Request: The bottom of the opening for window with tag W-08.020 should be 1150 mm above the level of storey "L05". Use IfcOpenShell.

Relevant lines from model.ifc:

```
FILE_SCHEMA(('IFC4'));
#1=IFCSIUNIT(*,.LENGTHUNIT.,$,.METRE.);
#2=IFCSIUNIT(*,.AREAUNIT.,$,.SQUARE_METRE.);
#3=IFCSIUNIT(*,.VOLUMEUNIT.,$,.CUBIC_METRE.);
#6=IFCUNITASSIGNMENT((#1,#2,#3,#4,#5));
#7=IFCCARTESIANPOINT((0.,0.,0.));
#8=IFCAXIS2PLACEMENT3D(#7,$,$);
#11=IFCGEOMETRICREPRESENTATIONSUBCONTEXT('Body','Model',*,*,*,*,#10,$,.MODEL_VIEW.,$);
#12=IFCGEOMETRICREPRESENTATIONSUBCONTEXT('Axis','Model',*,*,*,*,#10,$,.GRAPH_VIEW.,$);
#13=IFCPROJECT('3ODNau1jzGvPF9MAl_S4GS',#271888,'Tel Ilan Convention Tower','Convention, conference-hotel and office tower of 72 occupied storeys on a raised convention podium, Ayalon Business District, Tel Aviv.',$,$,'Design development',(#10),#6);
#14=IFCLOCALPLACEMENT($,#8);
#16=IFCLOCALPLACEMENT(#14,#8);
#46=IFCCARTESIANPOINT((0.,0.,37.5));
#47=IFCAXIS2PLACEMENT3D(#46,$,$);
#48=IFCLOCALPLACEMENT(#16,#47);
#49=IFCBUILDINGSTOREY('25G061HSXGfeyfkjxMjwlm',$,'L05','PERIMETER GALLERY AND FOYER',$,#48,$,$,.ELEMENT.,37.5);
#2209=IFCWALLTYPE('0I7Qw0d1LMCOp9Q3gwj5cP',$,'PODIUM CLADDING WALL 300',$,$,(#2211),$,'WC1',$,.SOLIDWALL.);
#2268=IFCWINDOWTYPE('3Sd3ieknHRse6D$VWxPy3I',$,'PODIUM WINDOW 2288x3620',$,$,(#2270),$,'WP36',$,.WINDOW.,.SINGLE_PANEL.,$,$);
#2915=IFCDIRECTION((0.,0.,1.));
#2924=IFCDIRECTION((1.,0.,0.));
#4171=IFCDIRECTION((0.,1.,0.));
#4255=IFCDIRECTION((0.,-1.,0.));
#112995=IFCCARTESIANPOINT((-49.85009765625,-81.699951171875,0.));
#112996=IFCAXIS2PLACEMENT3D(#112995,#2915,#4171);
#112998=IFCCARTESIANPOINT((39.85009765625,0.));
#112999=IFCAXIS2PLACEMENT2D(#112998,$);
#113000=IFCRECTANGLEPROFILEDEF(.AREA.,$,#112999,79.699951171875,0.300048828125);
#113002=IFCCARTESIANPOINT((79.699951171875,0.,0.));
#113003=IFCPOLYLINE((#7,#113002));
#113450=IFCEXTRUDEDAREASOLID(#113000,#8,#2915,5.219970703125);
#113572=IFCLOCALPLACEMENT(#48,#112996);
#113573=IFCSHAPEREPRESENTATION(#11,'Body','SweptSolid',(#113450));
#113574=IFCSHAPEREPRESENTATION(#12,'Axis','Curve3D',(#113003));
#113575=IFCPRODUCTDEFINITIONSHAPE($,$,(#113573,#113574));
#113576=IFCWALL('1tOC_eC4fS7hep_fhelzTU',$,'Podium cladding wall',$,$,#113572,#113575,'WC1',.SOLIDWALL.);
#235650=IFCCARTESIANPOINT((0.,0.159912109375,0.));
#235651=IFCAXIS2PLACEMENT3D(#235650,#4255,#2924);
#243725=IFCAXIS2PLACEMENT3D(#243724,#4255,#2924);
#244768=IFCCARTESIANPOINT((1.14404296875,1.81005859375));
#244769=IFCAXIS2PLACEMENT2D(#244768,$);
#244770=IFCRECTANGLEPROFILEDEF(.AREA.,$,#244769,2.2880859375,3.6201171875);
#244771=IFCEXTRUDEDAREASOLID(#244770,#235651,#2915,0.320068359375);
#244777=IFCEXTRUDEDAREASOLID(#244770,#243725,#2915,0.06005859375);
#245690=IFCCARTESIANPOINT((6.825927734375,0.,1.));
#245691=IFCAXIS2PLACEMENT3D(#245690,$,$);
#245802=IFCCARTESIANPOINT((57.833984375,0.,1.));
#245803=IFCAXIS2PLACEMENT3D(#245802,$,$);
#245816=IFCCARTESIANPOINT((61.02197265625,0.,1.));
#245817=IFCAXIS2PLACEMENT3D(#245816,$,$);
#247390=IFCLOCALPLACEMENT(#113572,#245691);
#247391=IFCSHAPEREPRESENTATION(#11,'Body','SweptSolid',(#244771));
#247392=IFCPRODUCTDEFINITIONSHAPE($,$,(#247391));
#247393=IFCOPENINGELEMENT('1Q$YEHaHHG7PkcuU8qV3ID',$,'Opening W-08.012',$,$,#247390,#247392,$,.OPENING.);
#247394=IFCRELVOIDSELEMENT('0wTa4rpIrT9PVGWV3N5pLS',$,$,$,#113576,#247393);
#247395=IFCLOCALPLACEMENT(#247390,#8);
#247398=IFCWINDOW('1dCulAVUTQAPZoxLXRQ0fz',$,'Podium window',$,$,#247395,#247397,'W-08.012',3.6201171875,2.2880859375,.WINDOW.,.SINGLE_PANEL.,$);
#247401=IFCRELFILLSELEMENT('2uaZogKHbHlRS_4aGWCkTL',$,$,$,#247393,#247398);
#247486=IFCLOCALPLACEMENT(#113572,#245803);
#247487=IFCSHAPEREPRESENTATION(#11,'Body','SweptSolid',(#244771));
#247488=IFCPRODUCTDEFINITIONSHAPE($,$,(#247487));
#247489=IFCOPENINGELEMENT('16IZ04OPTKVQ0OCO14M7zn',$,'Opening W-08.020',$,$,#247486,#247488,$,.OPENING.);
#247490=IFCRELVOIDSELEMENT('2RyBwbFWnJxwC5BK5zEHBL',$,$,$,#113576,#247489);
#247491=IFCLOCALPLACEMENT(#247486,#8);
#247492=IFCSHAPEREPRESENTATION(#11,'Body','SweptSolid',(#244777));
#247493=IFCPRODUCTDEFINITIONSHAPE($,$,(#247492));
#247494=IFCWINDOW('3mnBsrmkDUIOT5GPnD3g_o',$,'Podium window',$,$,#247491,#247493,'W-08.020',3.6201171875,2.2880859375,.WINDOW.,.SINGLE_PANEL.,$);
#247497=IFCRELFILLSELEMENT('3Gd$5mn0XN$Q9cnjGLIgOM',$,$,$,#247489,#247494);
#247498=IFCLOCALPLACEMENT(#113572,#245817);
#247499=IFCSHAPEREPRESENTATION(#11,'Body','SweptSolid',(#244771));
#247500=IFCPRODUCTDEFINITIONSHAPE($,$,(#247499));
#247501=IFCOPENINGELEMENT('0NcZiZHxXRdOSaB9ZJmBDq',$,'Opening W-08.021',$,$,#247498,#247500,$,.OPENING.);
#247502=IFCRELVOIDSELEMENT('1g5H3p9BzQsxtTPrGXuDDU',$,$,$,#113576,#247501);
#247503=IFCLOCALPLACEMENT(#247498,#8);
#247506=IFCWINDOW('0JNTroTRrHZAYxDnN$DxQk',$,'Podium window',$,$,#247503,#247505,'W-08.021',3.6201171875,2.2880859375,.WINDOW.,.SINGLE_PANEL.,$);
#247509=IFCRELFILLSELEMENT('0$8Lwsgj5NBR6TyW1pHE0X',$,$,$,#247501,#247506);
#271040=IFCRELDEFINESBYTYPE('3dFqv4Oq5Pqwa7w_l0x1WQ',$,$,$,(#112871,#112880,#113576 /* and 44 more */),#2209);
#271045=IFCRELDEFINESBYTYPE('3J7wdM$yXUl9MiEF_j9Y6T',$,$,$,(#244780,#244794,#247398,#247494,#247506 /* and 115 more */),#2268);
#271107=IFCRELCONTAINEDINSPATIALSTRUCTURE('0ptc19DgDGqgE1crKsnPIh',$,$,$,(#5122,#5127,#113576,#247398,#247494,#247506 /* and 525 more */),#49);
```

```python
import numpy as np
import ifcopenshell
import ifcopenshell.api.geometry
import ifcopenshell.geom
import ifcopenshell.util.element
import ifcopenshell.util.placement
import ifcopenshell.util.shape
import ifcopenshell.util.unit

model = ifcopenshell.open("model.ifc")
unit_scale = ifcopenshell.util.unit.calculate_unit_scale(model)

window = model.by_guid("3mnBsrmkDUIOT5GPnD3g_o")
opening = window.FillsVoids[0].RelatingOpeningElement
storey = ifcopenshell.util.element.get_container(window, ifc_class="IfcBuildingStorey")
level = ifcopenshell.util.placement.get_local_placement(storey.ObjectPlacement)[2, 3]

# The opening's origin need not be at the sill, so measure its lowest point.
shape = ifcopenshell.geom.create_shape(ifcopenshell.geom.settings(), opening)
bottom = ifcopenshell.util.shape.get_shape_bottom_elevation(shape, shape.geometry) / unit_scale
dz = level + 1.15 / unit_scale - bottom

shift = np.array([0.0, 0.0, dz])
# The window is placed relative to its opening, so it follows when the opening moves.
matrix = ifcopenshell.util.placement.get_local_placement(opening.ObjectPlacement)
matrix[:3, 3] += shift
ifcopenshell.api.geometry.edit_object_placement(
    model, product=opening, matrix=matrix, is_si=False, should_transform_children=True
)

print(f"moved by {dz * unit_scale:+.3f} m")

model.write("model-out.ifc")
```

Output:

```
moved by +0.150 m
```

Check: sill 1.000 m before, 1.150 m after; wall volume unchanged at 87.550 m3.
